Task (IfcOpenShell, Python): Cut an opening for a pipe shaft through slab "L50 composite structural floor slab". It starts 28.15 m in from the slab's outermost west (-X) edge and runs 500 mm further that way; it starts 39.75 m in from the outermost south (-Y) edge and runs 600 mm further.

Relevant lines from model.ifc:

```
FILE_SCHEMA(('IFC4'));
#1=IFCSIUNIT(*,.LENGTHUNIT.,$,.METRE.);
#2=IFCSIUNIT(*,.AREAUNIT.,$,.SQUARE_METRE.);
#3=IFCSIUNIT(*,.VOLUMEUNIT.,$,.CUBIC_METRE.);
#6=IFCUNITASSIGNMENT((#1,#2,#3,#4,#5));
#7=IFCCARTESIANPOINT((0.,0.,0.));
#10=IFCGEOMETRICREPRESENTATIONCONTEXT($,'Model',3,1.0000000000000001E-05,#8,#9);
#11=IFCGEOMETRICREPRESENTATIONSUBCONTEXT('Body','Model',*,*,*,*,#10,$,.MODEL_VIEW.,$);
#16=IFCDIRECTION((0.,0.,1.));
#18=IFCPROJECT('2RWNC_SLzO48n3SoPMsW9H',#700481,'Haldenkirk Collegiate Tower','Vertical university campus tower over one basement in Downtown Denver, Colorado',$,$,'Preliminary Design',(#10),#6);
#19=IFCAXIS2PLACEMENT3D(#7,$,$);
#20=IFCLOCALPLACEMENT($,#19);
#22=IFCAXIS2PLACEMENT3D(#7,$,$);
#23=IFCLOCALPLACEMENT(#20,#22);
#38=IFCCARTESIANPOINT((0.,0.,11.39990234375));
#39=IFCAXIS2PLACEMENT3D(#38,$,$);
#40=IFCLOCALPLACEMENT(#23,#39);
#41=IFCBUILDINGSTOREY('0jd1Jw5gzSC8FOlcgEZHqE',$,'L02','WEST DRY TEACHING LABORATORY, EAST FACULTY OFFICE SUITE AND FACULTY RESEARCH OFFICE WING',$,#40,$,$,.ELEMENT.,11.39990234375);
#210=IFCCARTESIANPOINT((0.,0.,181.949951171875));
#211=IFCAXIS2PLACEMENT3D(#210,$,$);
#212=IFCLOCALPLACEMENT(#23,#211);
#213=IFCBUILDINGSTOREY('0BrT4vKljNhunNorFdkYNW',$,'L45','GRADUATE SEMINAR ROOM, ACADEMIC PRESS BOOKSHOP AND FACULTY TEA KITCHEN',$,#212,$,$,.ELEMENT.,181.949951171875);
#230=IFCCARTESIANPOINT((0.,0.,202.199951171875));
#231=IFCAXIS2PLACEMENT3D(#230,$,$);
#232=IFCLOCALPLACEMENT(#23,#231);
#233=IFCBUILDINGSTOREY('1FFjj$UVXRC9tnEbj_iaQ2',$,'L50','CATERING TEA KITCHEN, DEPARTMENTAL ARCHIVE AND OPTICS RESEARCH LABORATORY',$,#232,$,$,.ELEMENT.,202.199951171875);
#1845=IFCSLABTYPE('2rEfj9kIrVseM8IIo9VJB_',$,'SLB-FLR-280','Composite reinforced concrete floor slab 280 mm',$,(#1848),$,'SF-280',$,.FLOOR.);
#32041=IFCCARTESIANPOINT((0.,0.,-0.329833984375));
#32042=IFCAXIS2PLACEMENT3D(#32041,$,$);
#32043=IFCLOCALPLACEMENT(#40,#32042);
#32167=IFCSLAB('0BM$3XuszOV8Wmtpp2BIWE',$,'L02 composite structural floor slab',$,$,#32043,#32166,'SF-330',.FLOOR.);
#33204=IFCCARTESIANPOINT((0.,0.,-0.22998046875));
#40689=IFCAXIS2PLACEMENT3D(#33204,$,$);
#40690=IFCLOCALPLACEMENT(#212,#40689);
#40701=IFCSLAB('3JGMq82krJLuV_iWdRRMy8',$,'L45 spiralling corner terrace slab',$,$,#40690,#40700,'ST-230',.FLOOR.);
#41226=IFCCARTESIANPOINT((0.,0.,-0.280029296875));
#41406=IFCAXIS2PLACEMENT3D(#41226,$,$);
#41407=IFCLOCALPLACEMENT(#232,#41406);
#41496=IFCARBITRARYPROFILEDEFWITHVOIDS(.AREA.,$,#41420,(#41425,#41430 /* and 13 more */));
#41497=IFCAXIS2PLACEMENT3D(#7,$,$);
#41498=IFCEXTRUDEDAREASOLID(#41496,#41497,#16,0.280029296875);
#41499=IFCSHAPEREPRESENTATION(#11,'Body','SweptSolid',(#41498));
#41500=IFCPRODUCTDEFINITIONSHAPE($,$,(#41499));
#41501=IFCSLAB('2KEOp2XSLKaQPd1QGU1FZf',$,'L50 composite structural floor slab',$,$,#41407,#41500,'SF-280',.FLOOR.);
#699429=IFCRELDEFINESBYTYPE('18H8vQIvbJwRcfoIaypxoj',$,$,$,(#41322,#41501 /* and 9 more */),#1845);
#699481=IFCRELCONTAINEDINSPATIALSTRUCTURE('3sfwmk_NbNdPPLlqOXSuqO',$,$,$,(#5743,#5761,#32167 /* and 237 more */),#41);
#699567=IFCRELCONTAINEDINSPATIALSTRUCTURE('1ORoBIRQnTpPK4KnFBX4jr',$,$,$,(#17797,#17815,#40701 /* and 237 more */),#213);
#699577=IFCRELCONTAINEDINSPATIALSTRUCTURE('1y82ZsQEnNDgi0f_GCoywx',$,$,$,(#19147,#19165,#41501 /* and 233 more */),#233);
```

```python
import numpy as np
import ifcopenshell
import ifcopenshell.api.feature
import ifcopenshell.api.geometry
import ifcopenshell.api.root
import ifcopenshell.geom
import ifcopenshell.util.placement
import ifcopenshell.util.representation
import ifcopenshell.util.shape
import ifcopenshell.util.unit

model = ifcopenshell.open("model.ifc")
unit_scale = ifcopenshell.util.unit.calculate_unit_scale(model)
settings = ifcopenshell.geom.settings()


def volume(element):
    """Net volume in cubic metres, openings subtracted."""
    shape = ifcopenshell.geom.create_shape(settings, element)
    return ifcopenshell.util.shape.get_volume(shape.geometry)


slab = model.by_guid("2KEOp2XSLKaQPd1QGU1FZf")
before = volume(slab)

# Extent in the slab's own axes, in metres. The edges named are its -X and -Y sides.
slab_shape = ifcopenshell.geom.create_shape(settings, slab)
vertices = ifcopenshell.util.shape.get_vertices(slab_shape.geometry)
x_min, y_min, bottom = vertices.min(axis=0)
top = vertices[:, 2].max()

opening = ifcopenshell.api.root.create_entity(model, ifc_class="IfcOpeningElement", name="Pipe shaft opening", predefined_type="OPENING")
context = ifcopenshell.util.representation.get_context(model, "Model", "Body", "MODEL_VIEW")
width, depth = 0.5, 0.6
outline = [(0.0, 0.0), (width, 0.0), (width, depth), (0.0, depth), (0.0, 0.0)]
# Overshoot both faces by 50 mm so the cut is clean.
shape = ifcopenshell.api.geometry.add_slab_representation(
    model, context=context, depth=top - bottom + 0.1, polyline=outline
)
ifcopenshell.api.geometry.assign_representation(model, product=opening, representation=shape)

matrix = ifcopenshell.util.placement.get_local_placement(slab.ObjectPlacement)
matrix[:, 3] = matrix @ np.append(np.array([x_min + 28.15, y_min + 39.75, bottom - 0.05]) / unit_scale, 1.0)
ifcopenshell.api.geometry.edit_object_placement(model, product=opening, matrix=matrix, is_si=False)
ifcopenshell.api.feature.add_feature(model, feature=opening, element=slab)

after = volume(slab)

print(f"slab volume {before:.3f} -> {after:.3f} m3")

model.write("model_updated.ifc")
```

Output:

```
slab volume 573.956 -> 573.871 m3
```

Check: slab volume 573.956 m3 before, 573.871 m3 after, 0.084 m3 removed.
